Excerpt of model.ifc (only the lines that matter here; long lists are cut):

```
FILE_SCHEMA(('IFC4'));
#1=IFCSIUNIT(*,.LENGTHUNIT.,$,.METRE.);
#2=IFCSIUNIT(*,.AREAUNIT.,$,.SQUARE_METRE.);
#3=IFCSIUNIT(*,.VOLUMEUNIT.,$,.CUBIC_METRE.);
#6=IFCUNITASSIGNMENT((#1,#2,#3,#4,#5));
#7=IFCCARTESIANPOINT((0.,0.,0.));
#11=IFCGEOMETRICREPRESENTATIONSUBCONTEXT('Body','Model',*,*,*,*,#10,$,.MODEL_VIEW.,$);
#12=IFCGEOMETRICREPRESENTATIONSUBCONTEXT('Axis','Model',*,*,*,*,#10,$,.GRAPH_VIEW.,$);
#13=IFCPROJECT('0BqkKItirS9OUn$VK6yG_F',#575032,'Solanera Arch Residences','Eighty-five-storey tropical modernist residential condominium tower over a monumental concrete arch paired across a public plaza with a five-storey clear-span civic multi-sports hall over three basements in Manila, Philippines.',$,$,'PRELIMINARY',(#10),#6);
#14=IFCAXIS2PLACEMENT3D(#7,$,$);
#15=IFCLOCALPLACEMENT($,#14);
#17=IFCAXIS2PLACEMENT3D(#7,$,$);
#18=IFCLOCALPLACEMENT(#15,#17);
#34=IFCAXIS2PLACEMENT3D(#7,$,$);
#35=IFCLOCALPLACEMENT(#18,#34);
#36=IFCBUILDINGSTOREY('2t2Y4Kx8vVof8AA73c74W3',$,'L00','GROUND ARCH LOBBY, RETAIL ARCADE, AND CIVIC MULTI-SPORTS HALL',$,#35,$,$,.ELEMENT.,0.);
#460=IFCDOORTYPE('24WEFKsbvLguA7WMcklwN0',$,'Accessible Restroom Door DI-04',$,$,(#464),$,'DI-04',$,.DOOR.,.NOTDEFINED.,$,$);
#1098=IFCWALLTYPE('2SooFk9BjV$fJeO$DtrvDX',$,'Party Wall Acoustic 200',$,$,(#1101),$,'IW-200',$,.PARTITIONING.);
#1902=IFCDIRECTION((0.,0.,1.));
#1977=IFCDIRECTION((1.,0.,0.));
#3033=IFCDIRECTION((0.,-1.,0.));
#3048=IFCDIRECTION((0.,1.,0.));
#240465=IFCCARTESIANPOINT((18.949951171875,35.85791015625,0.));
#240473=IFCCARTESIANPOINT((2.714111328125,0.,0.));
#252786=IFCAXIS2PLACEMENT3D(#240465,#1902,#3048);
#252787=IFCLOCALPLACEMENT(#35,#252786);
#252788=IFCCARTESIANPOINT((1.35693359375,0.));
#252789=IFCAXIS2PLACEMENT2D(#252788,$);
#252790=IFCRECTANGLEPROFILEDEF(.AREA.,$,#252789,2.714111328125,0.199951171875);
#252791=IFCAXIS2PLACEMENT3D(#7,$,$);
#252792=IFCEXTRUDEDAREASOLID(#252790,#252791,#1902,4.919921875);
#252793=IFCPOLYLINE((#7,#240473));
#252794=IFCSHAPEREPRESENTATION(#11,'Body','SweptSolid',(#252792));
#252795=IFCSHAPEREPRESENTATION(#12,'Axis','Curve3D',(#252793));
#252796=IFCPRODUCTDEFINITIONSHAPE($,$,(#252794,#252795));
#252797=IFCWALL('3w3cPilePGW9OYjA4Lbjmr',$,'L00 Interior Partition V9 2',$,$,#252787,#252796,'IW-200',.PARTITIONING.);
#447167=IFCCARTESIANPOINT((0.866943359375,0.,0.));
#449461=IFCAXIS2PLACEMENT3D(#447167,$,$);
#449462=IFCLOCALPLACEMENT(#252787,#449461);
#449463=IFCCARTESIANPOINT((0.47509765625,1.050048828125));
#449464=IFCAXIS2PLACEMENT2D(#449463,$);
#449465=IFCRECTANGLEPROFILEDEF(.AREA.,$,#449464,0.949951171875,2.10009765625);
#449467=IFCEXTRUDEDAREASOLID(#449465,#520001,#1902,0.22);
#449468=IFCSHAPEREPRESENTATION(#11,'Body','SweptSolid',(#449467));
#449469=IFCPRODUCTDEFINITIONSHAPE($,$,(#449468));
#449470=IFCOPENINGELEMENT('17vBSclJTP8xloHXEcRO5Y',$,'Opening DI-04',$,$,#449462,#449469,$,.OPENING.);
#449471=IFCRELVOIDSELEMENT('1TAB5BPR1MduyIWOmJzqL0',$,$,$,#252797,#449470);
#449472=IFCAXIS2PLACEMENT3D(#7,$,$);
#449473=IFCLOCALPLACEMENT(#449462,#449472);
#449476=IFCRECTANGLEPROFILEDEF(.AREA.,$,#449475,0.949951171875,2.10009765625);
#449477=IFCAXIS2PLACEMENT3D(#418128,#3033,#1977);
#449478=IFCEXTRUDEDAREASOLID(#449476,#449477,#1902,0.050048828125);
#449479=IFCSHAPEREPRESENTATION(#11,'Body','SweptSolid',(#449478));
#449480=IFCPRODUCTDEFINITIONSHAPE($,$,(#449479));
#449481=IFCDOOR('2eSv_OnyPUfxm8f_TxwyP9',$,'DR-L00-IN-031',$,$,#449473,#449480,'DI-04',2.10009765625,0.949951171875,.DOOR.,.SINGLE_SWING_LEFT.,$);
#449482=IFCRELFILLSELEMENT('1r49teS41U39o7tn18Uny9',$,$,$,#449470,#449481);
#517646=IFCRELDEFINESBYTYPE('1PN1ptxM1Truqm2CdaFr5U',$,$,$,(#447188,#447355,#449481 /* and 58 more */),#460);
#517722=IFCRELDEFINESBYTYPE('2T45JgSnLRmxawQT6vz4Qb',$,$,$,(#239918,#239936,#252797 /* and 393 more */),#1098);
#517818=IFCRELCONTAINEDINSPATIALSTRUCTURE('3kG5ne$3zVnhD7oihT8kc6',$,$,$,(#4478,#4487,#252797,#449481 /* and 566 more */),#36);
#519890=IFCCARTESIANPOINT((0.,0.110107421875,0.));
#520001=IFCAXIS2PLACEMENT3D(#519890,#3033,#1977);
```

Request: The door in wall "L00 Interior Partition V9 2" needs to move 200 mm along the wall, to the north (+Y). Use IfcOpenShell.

```python
import ifcopenshell
import ifcopenshell.api.geometry
import ifcopenshell.util.placement

model = ifcopenshell.open("model.ifc")

door = model.by_guid("2eSv_OnyPUfxm8f_TxwyP9")
opening = door.FillsVoids[0].RelatingOpeningElement
wall = opening.VoidsElements[0].RelatingBuildingElement

wall_matrix = ifcopenshell.util.placement.get_local_placement(wall.ObjectPlacement)
shift = wall_matrix[:3, 0] * 0.2
before = ifcopenshell.util.placement.get_local_placement(door.ObjectPlacement)[:3, 3].copy()

# The door is placed relative to its opening, so it follows when the opening moves.
matrix = ifcopenshell.util.placement.get_local_placement(opening.ObjectPlacement)
matrix[:3, 3] += shift
ifcopenshell.api.geometry.edit_object_placement(
    model, product=opening, matrix=matrix, is_si=False, should_transform_children=True
)

after = ifcopenshell.util.placement.get_local_placement(door.ObjectPlacement)[:3, 3]
print("door moved by", (after - before).round(3) + 0.0)

model.write("model_updated.ifc")
```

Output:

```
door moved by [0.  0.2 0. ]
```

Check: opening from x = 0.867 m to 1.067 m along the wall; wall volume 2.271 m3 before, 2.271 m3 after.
